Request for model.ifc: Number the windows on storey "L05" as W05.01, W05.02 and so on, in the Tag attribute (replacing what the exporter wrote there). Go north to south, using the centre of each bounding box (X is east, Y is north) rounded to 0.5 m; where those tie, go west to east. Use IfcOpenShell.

First a look at what the model holds.

```python
import ifcopenshell
import ifcopenshell.util.element
import ifcopenshell.util.placement

model = ifcopenshell.open("model.ifc")
print(model.schema)
storey = next(s for s in model.by_type("IfcBuildingStorey") if s.Name == "L05")
windows = [e for e in ifcopenshell.util.element.get_decomposition(storey) if e.is_a("IfcWindow")]
for e in sorted(windows, key=lambda e: e.id()):
    origin = ifcopenshell.util.placement.get_local_placement(e.ObjectPlacement)[:3, 3]
    print(e.id(), e.Tag, e.Name, origin.round(2) + 0.0, sep=" | ")
```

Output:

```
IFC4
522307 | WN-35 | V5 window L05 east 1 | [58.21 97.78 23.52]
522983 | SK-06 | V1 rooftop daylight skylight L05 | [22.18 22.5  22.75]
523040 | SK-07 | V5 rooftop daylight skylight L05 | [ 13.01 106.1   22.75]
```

```python
import ifcopenshell
import ifcopenshell.geom
import ifcopenshell.util.element
import ifcopenshell.util.shape

model = ifcopenshell.open("model.ifc")
settings = ifcopenshell.geom.settings()
settings.set("use-world-coords", True)


def centre(element):
    shape = ifcopenshell.geom.create_shape(settings, element)
    return ifcopenshell.util.shape.get_bbox_centroid(shape.geometry)


storey = next(s for s in model.by_type("IfcBuildingStorey") if s.Name == "L05")
windows = [e for e in ifcopenshell.util.element.get_decomposition(storey) if e.is_a("IfcWindow")]

# Insertion points can sit at a corner or the storey origin, so sort by the geometry (in metres).
centres = {e: centre(e) for e in windows}
windows.sort(key=lambda e: (-round(centres[e][1] / 0.5), centres[e][0]))

for i, e in enumerate(windows, start=1):
    number = f"W05.{i:02d}"
    e.Tag = number
    print(e.id(), number)

model.write("model_v2.ifc")
```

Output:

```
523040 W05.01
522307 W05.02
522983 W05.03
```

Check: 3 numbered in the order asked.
